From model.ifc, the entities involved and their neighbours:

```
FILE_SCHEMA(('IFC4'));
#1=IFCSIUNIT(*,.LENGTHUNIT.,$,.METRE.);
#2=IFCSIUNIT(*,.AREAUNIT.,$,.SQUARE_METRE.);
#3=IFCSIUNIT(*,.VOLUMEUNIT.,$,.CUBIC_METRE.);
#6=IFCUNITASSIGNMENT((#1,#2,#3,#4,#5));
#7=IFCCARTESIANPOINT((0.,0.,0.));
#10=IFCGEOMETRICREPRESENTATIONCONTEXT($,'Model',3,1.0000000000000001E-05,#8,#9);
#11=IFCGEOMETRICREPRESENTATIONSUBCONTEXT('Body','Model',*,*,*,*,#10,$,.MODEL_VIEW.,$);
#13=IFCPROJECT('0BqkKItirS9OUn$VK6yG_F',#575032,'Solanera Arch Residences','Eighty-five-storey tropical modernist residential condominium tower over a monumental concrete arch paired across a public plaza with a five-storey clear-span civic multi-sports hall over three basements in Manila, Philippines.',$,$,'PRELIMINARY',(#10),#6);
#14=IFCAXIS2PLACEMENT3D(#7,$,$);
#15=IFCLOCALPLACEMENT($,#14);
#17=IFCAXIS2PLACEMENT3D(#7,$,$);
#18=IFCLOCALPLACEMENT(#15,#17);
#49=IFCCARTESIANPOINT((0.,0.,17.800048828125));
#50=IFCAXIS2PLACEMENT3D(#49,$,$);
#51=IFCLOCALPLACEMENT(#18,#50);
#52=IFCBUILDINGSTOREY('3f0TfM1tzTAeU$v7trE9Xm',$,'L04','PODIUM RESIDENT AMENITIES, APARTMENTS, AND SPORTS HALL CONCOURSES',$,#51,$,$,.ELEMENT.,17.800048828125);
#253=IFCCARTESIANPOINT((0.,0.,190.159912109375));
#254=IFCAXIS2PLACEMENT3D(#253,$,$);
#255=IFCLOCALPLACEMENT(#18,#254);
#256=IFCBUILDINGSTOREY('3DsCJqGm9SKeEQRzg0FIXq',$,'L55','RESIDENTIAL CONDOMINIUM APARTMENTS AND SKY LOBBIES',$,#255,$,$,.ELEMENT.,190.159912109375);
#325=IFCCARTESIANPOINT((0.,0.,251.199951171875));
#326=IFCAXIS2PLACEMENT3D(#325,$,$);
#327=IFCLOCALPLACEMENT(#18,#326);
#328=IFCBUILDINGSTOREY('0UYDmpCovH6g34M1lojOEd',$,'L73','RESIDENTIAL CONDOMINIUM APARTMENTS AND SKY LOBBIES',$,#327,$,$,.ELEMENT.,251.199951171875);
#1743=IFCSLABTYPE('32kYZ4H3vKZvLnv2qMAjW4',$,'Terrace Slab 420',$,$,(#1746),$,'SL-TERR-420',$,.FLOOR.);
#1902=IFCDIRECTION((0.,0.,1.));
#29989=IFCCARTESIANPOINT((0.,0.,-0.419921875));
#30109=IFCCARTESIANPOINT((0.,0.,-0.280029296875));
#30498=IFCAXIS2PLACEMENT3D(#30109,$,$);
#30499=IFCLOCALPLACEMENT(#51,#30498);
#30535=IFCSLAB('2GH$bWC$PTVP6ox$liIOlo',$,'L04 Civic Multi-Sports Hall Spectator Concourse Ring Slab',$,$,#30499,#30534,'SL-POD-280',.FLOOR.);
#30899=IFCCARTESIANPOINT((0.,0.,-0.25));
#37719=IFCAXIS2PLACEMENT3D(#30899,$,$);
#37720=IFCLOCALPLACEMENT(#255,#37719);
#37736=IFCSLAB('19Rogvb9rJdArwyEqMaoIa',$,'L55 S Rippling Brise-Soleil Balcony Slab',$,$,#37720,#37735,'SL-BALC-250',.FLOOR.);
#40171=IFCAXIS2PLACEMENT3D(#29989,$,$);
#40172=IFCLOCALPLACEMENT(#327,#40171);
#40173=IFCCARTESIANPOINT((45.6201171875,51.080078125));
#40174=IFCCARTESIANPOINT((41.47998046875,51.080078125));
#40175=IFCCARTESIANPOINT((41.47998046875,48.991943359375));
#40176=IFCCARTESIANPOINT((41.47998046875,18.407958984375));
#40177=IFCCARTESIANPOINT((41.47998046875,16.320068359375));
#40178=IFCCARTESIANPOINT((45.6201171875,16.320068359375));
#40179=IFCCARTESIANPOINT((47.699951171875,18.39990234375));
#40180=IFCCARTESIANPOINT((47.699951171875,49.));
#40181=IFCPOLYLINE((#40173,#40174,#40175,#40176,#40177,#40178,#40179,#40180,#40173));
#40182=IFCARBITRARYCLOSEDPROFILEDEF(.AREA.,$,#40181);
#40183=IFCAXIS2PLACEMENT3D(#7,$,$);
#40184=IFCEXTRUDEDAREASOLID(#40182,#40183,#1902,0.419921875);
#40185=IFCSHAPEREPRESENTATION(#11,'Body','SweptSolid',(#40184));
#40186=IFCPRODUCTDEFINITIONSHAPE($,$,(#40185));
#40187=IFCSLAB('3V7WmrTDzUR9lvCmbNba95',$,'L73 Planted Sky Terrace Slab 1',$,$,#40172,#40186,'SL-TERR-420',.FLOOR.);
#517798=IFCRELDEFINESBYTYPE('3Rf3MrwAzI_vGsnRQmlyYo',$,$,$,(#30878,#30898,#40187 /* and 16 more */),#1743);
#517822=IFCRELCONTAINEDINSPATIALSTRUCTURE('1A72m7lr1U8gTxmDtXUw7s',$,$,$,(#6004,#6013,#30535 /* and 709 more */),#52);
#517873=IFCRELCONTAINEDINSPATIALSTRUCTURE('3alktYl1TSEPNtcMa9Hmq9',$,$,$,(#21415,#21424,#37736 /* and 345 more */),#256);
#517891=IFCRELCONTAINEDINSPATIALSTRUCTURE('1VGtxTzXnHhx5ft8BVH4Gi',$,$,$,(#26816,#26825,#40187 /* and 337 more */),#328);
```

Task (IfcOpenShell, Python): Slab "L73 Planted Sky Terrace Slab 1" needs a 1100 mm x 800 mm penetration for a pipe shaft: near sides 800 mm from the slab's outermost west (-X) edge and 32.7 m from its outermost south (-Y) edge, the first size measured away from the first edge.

```python
import numpy as np
import ifcopenshell
import ifcopenshell.api.feature
import ifcopenshell.api.geometry
import ifcopenshell.api.root
import ifcopenshell.geom
import ifcopenshell.util.placement
import ifcopenshell.util.representation
import ifcopenshell.util.shape
import ifcopenshell.util.unit

model = ifcopenshell.open("model.ifc")
unit_scale = ifcopenshell.util.unit.calculate_unit_scale(model)
settings = ifcopenshell.geom.settings()


def volume(element):
    """Net volume in cubic metres, openings subtracted."""
    shape = ifcopenshell.geom.create_shape(settings, element)
    return ifcopenshell.util.shape.get_volume(shape.geometry)


slab = model.by_id(40187)
before = volume(slab)

# Extent in the slab's own axes, in metres. The edges named are its -X and -Y sides.
slab_shape = ifcopenshell.geom.create_shape(settings, slab)
vertices = ifcopenshell.util.shape.get_vertices(slab_shape.geometry)
x_min, y_min, bottom = vertices.min(axis=0)
top = vertices[:, 2].max()

opening = ifcopenshell.api.root.create_entity(model, ifc_class="IfcOpeningElement", name="Pipe shaft opening", predefined_type="OPENING")
context = ifcopenshell.util.representation.get_context(model, "Model", "Body", "MODEL_VIEW")
width, depth = 1.1, 0.8
outline = [(0.0, 0.0), (width, 0.0), (width, depth), (0.0, depth), (0.0, 0.0)]
# Overshoot both faces by 50 mm so the cut is clean.
shape = ifcopenshell.api.geometry.add_slab_representation(
    model, context=context, depth=top - bottom + 0.1, polyline=outline
)
ifcopenshell.api.geometry.assign_representation(model, product=opening, representation=shape)

matrix = ifcopenshell.util.placement.get_local_placement(slab.ObjectPlacement)
matrix[:, 3] = matrix @ np.append(np.array([x_min + 0.8, y_min + 32.7, bottom - 0.05]) / unit_scale, 1.0)
ifcopenshell.api.geometry.edit_object_placement(model, product=opening, matrix=matrix, is_si=False)
ifcopenshell.api.feature.add_feature(model, feature=opening, element=slab)

after = volume(slab)

print(f"slab volume {before:.3f} -> {after:.3f} m3")

model.write("model-out.ifc")
```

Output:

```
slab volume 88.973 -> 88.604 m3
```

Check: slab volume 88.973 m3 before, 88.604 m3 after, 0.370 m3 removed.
